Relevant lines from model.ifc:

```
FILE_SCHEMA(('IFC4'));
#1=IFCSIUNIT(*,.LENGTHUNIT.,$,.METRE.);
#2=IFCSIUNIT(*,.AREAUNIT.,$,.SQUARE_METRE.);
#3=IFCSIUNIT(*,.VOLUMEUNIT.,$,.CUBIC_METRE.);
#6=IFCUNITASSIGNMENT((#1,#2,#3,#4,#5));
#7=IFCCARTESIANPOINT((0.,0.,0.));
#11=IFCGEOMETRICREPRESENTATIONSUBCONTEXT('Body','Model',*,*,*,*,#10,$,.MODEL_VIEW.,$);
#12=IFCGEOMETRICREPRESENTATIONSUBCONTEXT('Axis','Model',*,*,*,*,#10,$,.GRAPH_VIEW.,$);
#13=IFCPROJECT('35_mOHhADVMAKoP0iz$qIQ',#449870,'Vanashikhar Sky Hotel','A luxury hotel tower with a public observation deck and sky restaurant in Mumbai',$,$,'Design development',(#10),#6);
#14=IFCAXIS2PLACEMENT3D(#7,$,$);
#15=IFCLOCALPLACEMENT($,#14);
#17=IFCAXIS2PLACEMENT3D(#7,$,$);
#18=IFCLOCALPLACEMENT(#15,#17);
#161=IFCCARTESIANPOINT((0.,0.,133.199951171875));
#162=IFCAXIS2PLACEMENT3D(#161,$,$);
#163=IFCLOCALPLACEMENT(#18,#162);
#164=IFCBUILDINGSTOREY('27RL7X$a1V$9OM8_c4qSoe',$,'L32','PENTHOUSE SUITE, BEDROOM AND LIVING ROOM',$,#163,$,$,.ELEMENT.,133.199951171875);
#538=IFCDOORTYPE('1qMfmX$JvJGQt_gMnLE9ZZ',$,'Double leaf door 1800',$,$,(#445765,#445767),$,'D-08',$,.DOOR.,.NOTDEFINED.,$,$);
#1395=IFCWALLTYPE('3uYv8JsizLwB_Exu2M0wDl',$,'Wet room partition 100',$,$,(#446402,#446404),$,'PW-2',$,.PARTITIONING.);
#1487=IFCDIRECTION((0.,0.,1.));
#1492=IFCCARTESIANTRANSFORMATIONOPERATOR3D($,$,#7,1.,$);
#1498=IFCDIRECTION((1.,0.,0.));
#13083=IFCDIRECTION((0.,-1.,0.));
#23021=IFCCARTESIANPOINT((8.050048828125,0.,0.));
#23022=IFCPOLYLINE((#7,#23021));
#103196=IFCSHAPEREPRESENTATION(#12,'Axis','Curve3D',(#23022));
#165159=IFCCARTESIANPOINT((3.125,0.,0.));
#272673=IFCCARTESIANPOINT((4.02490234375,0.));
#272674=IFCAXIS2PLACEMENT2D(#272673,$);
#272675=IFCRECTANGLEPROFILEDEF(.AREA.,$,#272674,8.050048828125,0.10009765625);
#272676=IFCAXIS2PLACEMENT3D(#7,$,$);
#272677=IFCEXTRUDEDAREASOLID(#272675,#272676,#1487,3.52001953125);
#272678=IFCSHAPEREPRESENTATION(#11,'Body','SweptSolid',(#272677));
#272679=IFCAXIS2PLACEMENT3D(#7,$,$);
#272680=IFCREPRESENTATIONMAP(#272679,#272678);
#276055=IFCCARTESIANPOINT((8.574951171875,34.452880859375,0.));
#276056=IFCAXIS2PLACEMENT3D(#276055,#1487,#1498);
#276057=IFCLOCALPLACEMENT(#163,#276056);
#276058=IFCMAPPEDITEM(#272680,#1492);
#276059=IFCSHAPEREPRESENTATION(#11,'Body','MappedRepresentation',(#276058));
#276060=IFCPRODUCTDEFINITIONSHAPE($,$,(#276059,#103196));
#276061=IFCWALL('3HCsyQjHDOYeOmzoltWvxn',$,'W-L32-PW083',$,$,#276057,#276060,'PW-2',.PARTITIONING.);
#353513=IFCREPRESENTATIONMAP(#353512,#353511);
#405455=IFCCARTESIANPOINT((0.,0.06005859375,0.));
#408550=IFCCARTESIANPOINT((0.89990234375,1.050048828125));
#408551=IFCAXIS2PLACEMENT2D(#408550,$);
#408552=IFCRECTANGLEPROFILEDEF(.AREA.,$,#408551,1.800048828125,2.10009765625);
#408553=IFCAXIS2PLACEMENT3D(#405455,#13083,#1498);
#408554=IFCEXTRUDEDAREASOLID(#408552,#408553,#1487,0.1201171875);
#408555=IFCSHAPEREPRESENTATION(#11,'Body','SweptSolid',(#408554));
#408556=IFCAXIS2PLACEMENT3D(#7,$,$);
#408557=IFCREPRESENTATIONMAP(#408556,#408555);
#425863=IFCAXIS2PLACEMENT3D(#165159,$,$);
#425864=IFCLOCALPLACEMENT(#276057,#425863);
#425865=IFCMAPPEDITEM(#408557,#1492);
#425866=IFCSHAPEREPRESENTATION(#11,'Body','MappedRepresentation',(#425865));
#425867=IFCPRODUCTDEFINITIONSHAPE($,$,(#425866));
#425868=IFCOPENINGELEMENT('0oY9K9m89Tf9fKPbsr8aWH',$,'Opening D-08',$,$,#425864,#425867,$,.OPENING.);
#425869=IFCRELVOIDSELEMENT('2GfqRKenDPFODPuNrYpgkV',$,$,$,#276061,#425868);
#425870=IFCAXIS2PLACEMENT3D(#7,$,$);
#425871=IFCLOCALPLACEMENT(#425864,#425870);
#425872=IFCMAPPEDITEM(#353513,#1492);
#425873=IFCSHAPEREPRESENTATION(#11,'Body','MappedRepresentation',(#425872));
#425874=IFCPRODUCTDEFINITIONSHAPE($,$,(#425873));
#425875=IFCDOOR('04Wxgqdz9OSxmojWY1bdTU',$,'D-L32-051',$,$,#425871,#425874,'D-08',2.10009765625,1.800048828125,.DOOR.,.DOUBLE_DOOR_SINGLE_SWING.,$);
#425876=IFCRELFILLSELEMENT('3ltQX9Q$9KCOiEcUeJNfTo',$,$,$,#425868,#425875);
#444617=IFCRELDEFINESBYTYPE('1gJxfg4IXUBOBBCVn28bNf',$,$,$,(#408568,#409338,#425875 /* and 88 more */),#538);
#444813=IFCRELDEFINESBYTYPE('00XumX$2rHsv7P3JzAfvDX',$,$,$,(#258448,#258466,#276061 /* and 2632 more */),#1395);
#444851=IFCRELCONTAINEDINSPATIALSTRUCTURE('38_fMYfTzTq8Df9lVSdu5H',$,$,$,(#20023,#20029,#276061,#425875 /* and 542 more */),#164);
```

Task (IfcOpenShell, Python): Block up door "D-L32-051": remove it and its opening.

```python
import ifcopenshell
import ifcopenshell.api.feature
import ifcopenshell.api.root
import ifcopenshell.geom
import ifcopenshell.util.shape

model = ifcopenshell.open("model.ifc")
settings = ifcopenshell.geom.settings()


def volume(element):
    """Net volume in cubic metres, openings subtracted."""
    shape = ifcopenshell.geom.create_shape(settings, element)
    return ifcopenshell.util.shape.get_volume(shape.geometry)


door = model.by_id(425875)
opening = door.FillsVoids[0].RelatingOpeningElement
wall = opening.VoidsElements[0].RelatingBuildingElement
before = volume(wall)

ifcopenshell.api.root.remove_product(model, product=door)
ifcopenshell.api.feature.remove_feature(model, feature=opening)

after = volume(wall)

print(f"wall volume {before:.3f} -> {after:.3f} m3")

model.write("model_v2.ifc")
```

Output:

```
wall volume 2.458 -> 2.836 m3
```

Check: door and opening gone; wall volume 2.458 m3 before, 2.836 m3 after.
